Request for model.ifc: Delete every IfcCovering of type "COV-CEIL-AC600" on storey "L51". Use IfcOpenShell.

First a look at what the model holds.

```python
import ifcopenshell
import ifcopenshell.util.element

model = ifcopenshell.open("model.ifc")
print(model.schema)
storey = next(s for s in model.by_type("IfcBuildingStorey") if s.Name == "L51")
coverings = [e for e in ifcopenshell.util.element.get_decomposition(storey) if e.is_a("IfcCovering")]
seen = {}
for e in coverings:
    element_type = ifcopenshell.util.element.get_type(e)
    name = element_type.Name if element_type not in (None, e) else None
    seen[name] = seen.get(name, 0) + 1
for name, count in sorted(seen.items(), key=str):
    print(count, "x", name)
```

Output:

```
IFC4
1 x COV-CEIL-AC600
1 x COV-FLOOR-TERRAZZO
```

```python
import ifcopenshell
import ifcopenshell.api.root
import ifcopenshell.util.element

model = ifcopenshell.open("model.ifc")

storey = next(s for s in model.by_type("IfcBuildingStorey") if s.Name == "L51")
coverings = [e for e in ifcopenshell.util.element.get_decomposition(storey) if e.is_a("IfcCovering")]
targets = [e for e in coverings if (t := ifcopenshell.util.element.get_type(e)) not in (None, e) and t.Name == "COV-CEIL-AC600"]

for e in targets:
    ifcopenshell.api.root.remove_product(model, product=e)
print(len(targets), "removed")

model.write("model_updated.ifc")
```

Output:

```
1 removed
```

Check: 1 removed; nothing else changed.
